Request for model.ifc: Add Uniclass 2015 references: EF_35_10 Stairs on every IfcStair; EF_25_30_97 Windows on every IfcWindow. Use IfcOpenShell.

First a look at what the model holds.

```python
import ifcopenshell

model = ifcopenshell.open("model.ifc")
print(model.schema)
print("classifications:", [c.Name for c in model.by_type("IfcClassification")])
for ifc_class in ("IfcDoor", "IfcRoof", "IfcStair", "IfcWall", "IfcWindow"):
    print(ifc_class, len(model.by_type(ifc_class)))
```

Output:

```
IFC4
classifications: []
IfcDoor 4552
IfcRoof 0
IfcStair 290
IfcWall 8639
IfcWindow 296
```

```python
import ifcopenshell
import ifcopenshell.api.classification

model = ifcopenshell.open("model.ifc")

system = ifcopenshell.api.classification.add_classification(model, classification="Uniclass 2015")

codes = {
    "IfcStair": ("EF_35_10", "Stairs"),
    "IfcWindow": ("EF_25_30_97", "Windows"),
}
for ifc_class, (code, name) in codes.items():
    products = model.by_type(ifc_class)
    ifcopenshell.api.classification.add_reference(
        model, products=products, classification=system, identification=code, name=name
    )
    print(code, len(products))

model.write("model_edited.ifc")
```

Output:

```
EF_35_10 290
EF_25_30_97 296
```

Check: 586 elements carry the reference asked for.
